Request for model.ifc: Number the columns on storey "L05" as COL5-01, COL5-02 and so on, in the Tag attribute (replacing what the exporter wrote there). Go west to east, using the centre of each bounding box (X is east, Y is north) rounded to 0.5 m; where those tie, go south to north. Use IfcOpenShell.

First a look at what the model holds.

```python
import ifcopenshell
import ifcopenshell.util.element
import ifcopenshell.util.placement

model = ifcopenshell.open("model.ifc")
print(model.schema)
storey = next(s for s in model.by_type("IfcBuildingStorey") if s.Name == "L05")
columns = [e for e in ifcopenshell.util.element.get_decomposition(storey) if e.is_a("IfcColumn")]
for e in sorted(columns, key=lambda e: e.id()):
    origin = ifcopenshell.util.placement.get_local_placement(e.ObjectPlacement)[:3, 3]
    print(e.id(), e.Tag, e.Name, origin.round(2) + 0.0, sep=" | ")
```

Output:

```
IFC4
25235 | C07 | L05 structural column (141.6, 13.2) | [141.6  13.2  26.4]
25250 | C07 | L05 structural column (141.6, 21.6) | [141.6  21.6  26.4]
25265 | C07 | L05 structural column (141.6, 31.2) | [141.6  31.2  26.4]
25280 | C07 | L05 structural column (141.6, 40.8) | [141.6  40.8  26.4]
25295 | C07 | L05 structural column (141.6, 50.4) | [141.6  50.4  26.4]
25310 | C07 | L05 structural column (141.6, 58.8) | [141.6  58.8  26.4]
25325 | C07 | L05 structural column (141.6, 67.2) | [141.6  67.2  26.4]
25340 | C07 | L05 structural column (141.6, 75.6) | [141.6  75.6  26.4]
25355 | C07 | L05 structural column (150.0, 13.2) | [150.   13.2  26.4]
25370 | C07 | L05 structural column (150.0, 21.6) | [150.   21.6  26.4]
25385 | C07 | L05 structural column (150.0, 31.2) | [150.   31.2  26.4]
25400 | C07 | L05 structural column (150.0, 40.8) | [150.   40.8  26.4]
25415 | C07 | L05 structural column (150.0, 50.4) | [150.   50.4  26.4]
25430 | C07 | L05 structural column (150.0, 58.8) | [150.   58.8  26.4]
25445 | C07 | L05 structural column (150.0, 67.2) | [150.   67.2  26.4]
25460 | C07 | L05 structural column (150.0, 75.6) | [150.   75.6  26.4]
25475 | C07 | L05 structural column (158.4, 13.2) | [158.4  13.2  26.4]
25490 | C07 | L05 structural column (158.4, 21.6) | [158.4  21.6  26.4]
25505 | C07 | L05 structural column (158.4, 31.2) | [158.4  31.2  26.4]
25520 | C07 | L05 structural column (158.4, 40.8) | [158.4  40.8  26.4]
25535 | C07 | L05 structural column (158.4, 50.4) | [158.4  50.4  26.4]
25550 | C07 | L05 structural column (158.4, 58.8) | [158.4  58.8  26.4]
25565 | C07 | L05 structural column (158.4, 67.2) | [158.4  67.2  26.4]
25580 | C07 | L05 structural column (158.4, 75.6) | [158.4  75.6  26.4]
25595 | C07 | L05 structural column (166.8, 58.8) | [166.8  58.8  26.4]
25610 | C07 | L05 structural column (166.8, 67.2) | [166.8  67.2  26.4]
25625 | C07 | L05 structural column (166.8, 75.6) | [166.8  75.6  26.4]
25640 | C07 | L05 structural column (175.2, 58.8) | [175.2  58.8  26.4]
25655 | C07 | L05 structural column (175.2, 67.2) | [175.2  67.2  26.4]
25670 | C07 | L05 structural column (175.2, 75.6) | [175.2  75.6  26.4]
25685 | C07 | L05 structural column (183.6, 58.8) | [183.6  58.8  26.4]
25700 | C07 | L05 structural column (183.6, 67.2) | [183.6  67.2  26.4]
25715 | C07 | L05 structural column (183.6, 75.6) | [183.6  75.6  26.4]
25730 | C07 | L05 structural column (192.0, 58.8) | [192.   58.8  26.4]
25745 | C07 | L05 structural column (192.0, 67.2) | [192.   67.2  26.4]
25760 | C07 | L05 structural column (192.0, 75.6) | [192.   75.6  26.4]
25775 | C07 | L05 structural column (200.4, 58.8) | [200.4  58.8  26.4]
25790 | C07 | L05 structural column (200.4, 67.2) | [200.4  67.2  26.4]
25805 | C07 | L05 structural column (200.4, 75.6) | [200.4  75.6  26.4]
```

```python
import ifcopenshell
import ifcopenshell.geom
import ifcopenshell.util.element
import ifcopenshell.util.shape

model = ifcopenshell.open("model.ifc")
settings = ifcopenshell.geom.settings()
settings.set("use-world-coords", True)


def centre(element):
    shape = ifcopenshell.geom.create_shape(settings, element)
    return ifcopenshell.util.shape.get_bbox_centroid(shape.geometry)


storey = next(s for s in model.by_type("IfcBuildingStorey") if s.Name == "L05")
columns = [e for e in ifcopenshell.util.element.get_decomposition(storey) if e.is_a("IfcColumn")]

# Insertion points can sit at a corner or the storey origin, so sort by the geometry (in metres).
centres = {e: centre(e) for e in columns}
columns.sort(key=lambda e: (round(centres[e][0] / 0.5), centres[e][1]))

for i, e in enumerate(columns, start=1):
    number = f"COL5-{i:02d}"
    e.Tag = number
    print(e.id(), number)

model.write("model_rev.ifc")
```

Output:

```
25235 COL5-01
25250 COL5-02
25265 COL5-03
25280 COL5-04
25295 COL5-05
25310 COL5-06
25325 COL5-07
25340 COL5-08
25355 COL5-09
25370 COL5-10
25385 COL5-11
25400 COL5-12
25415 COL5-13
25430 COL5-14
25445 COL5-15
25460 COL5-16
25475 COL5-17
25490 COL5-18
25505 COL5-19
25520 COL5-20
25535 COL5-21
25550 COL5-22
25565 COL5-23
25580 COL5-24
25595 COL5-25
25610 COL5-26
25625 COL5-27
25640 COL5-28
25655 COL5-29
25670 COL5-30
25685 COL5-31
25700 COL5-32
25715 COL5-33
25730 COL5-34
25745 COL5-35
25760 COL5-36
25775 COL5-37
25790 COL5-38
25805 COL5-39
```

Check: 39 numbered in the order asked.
